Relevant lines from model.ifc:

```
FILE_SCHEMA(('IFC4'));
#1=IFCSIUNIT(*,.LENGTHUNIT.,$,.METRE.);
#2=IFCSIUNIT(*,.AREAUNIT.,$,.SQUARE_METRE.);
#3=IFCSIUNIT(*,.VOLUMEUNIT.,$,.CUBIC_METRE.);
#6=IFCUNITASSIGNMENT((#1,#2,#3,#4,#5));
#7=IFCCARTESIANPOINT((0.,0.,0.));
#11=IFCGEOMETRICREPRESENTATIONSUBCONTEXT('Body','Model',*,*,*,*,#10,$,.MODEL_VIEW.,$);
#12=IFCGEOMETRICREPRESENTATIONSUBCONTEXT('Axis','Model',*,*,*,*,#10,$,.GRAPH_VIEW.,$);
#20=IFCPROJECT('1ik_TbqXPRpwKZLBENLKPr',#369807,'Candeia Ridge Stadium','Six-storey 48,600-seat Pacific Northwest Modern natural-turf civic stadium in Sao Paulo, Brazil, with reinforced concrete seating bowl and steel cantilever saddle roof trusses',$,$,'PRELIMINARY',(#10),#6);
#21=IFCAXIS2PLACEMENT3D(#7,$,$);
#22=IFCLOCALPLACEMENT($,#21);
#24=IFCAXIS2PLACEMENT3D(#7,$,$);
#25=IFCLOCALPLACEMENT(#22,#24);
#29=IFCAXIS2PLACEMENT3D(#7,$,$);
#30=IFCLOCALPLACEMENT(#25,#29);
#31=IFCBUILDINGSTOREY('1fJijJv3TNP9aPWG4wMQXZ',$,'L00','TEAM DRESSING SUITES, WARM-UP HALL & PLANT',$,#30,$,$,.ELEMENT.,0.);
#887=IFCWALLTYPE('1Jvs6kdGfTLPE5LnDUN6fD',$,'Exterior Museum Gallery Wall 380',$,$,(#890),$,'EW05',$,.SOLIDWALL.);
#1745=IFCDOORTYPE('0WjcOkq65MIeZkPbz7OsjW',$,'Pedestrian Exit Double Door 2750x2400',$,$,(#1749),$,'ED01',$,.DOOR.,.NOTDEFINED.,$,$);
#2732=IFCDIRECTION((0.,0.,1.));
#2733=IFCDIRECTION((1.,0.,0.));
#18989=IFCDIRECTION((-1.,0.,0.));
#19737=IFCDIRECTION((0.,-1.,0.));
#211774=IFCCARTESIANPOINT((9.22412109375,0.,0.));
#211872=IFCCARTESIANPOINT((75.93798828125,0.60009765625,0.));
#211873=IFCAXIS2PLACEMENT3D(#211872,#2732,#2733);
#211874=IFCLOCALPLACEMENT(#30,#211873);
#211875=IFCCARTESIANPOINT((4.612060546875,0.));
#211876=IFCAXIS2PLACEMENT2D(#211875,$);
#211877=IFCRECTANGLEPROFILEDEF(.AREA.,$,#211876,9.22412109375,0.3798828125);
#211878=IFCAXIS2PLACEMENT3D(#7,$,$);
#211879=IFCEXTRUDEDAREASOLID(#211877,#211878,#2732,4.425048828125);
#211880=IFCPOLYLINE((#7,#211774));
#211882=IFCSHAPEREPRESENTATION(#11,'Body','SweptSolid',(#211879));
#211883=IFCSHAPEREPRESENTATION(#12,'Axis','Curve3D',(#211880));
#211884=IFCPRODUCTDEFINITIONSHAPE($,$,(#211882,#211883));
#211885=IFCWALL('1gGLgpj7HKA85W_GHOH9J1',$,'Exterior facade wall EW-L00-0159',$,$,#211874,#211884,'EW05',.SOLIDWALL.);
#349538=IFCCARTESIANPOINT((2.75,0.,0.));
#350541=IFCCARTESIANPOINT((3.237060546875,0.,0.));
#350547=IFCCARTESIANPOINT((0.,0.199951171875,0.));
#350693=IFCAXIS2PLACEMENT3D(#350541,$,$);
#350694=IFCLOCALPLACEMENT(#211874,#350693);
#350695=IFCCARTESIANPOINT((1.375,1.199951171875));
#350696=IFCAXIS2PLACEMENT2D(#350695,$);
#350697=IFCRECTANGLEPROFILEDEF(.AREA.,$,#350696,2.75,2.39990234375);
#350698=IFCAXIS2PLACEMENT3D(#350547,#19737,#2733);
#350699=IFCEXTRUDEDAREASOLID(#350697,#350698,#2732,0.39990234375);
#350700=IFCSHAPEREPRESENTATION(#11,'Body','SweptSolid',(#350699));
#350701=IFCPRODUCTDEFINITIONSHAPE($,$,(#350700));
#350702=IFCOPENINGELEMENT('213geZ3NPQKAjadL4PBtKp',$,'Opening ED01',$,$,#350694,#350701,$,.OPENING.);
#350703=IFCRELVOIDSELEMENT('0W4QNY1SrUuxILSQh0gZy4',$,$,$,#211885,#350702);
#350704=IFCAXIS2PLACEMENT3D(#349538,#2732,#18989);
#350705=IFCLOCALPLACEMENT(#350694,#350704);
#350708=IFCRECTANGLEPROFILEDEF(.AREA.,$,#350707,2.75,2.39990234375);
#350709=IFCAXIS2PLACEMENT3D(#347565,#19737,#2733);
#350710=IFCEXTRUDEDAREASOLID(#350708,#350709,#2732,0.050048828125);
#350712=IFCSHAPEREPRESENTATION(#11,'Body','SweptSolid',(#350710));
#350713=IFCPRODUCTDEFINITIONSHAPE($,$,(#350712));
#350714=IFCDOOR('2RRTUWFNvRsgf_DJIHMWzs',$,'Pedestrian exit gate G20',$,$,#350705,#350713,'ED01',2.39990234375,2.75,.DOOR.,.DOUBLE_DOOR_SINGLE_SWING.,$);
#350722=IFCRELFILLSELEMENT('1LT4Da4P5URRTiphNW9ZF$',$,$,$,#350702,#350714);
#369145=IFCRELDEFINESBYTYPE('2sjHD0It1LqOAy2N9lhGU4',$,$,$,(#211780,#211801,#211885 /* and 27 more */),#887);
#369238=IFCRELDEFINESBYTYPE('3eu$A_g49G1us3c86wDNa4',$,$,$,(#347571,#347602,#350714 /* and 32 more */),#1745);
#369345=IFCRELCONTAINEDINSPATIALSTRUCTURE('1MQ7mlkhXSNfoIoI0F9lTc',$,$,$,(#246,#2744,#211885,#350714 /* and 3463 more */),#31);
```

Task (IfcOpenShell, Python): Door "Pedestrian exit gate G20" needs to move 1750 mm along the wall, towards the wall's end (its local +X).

```python
import ifcopenshell
import ifcopenshell.api.geometry
import ifcopenshell.util.placement

model = ifcopenshell.open("model.ifc")

door = model.by_guid("2RRTUWFNvRsgf_DJIHMWzs")
opening = door.FillsVoids[0].RelatingOpeningElement
wall = opening.VoidsElements[0].RelatingBuildingElement

wall_matrix = ifcopenshell.util.placement.get_local_placement(wall.ObjectPlacement)
shift = wall_matrix[:3, 0] * 1.75
before = ifcopenshell.util.placement.get_local_placement(door.ObjectPlacement)[:3, 3].copy()

# The door is placed relative to its opening, so it follows when the opening moves.
matrix = ifcopenshell.util.placement.get_local_placement(opening.ObjectPlacement)
matrix[:3, 3] += shift
ifcopenshell.api.geometry.edit_object_placement(
    model, product=opening, matrix=matrix, is_si=False, should_transform_children=True
)

after = ifcopenshell.util.placement.get_local_placement(door.ObjectPlacement)[:3, 3]
print("door moved by", (after - before).round(3) + 0.0)

model.write("model_updated.ifc")
```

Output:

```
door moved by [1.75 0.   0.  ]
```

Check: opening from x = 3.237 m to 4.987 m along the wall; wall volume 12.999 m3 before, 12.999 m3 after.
